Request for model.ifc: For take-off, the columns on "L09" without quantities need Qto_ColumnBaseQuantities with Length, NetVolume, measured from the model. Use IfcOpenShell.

First a look at what the model holds.

```python
import ifcopenshell
import ifcopenshell.util.element
import ifcopenshell.util.unit

model = ifcopenshell.open("model.ifc")
print(model.schema)
for unit_type in ("LENGTHUNIT", "AREAUNIT", "VOLUMEUNIT"):
    print(unit_type, ifcopenshell.util.unit.calculate_unit_scale(model, unit_type))
storey = next(s for s in model.by_type("IfcBuildingStorey") if s.Name == "L09")
columns = [e for e in ifcopenshell.util.element.get_decomposition(storey) if e.is_a("IfcColumn")]
for e in sorted(columns, key=lambda e: e.id()):
    print(e.id(), e.is_a(), e.Name, list(ifcopenshell.util.element.get_psets(e, qtos_only=True)), sep=" | ")
```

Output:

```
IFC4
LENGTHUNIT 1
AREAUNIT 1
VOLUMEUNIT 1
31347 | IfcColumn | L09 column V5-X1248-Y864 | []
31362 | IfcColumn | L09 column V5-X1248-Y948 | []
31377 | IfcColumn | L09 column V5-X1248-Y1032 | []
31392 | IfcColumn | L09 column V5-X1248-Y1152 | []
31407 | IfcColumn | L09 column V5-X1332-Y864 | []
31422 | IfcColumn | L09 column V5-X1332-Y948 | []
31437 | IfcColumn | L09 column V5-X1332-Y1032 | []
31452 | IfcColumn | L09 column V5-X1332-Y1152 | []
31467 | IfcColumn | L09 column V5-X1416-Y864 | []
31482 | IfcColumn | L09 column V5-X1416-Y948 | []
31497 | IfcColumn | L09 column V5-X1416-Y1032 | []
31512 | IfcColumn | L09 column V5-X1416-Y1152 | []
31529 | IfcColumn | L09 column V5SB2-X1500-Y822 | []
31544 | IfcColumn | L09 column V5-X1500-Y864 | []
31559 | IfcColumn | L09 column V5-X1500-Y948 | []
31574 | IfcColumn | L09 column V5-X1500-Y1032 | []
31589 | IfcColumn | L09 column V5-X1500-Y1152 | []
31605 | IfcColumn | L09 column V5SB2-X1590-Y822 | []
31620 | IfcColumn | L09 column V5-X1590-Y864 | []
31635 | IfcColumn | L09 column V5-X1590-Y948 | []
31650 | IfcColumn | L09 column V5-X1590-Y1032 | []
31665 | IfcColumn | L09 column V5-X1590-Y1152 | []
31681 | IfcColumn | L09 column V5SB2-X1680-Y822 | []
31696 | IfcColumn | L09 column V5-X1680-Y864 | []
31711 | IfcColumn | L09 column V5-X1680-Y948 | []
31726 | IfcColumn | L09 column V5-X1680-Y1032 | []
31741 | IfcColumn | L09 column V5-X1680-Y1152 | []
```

```python
import ifcopenshell
import ifcopenshell.api.pset
import ifcopenshell.geom
import ifcopenshell.util.element
import ifcopenshell.util.shape
import ifcopenshell.util.unit

model = ifcopenshell.open("model.ifc")
unit_scale = ifcopenshell.util.unit.calculate_unit_scale(model)
volume_scale = ifcopenshell.util.unit.calculate_unit_scale(model, "VOLUMEUNIT")
settings = ifcopenshell.geom.settings()

storey = next(s for s in model.by_type("IfcBuildingStorey") if s.Name == "L09")
columns = [e for e in ifcopenshell.util.element.get_decomposition(storey) if e.is_a("IfcColumn")]

for e in sorted(columns, key=lambda e: e.id()):
    if ifcopenshell.util.element.get_psets(e, qtos_only=True, should_inherit=False):
        continue
    # Geometry comes back in metres, in the element's own axes.
    shape = ifcopenshell.geom.create_shape(settings, e)
    values = {
        "Length": ifcopenshell.util.shape.get_z(shape.geometry) / unit_scale,
        "NetVolume": ifcopenshell.util.shape.get_volume(shape.geometry) / volume_scale,
    }
    qto = ifcopenshell.api.pset.add_qto(model, product=e, name="Qto_ColumnBaseQuantities")
    ifcopenshell.api.pset.edit_qto(model, qto=qto, properties=values)
    print(e.id(), {k: round(v, 3) for k, v in values.items()})

model.write("model_rev.ifc")
```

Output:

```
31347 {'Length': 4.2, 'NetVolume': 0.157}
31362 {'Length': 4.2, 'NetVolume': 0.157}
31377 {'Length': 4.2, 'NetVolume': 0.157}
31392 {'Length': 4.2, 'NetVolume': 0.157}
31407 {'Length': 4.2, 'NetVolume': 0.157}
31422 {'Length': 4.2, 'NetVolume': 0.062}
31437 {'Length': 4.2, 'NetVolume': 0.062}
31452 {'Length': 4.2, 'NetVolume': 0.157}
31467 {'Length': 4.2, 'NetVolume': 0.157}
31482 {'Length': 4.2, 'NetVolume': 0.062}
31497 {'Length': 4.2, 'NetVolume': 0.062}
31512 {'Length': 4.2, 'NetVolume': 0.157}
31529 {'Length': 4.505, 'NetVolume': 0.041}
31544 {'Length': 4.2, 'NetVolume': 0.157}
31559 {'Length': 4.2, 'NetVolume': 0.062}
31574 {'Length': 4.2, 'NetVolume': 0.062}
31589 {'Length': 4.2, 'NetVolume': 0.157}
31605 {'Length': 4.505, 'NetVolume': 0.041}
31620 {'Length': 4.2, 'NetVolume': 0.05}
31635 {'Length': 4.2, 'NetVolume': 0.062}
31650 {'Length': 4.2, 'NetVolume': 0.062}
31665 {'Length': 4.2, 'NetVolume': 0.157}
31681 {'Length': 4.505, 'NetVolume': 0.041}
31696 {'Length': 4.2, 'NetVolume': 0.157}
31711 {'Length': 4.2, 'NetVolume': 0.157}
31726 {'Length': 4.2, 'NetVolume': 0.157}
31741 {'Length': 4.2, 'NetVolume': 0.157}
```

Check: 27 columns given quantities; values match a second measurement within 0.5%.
